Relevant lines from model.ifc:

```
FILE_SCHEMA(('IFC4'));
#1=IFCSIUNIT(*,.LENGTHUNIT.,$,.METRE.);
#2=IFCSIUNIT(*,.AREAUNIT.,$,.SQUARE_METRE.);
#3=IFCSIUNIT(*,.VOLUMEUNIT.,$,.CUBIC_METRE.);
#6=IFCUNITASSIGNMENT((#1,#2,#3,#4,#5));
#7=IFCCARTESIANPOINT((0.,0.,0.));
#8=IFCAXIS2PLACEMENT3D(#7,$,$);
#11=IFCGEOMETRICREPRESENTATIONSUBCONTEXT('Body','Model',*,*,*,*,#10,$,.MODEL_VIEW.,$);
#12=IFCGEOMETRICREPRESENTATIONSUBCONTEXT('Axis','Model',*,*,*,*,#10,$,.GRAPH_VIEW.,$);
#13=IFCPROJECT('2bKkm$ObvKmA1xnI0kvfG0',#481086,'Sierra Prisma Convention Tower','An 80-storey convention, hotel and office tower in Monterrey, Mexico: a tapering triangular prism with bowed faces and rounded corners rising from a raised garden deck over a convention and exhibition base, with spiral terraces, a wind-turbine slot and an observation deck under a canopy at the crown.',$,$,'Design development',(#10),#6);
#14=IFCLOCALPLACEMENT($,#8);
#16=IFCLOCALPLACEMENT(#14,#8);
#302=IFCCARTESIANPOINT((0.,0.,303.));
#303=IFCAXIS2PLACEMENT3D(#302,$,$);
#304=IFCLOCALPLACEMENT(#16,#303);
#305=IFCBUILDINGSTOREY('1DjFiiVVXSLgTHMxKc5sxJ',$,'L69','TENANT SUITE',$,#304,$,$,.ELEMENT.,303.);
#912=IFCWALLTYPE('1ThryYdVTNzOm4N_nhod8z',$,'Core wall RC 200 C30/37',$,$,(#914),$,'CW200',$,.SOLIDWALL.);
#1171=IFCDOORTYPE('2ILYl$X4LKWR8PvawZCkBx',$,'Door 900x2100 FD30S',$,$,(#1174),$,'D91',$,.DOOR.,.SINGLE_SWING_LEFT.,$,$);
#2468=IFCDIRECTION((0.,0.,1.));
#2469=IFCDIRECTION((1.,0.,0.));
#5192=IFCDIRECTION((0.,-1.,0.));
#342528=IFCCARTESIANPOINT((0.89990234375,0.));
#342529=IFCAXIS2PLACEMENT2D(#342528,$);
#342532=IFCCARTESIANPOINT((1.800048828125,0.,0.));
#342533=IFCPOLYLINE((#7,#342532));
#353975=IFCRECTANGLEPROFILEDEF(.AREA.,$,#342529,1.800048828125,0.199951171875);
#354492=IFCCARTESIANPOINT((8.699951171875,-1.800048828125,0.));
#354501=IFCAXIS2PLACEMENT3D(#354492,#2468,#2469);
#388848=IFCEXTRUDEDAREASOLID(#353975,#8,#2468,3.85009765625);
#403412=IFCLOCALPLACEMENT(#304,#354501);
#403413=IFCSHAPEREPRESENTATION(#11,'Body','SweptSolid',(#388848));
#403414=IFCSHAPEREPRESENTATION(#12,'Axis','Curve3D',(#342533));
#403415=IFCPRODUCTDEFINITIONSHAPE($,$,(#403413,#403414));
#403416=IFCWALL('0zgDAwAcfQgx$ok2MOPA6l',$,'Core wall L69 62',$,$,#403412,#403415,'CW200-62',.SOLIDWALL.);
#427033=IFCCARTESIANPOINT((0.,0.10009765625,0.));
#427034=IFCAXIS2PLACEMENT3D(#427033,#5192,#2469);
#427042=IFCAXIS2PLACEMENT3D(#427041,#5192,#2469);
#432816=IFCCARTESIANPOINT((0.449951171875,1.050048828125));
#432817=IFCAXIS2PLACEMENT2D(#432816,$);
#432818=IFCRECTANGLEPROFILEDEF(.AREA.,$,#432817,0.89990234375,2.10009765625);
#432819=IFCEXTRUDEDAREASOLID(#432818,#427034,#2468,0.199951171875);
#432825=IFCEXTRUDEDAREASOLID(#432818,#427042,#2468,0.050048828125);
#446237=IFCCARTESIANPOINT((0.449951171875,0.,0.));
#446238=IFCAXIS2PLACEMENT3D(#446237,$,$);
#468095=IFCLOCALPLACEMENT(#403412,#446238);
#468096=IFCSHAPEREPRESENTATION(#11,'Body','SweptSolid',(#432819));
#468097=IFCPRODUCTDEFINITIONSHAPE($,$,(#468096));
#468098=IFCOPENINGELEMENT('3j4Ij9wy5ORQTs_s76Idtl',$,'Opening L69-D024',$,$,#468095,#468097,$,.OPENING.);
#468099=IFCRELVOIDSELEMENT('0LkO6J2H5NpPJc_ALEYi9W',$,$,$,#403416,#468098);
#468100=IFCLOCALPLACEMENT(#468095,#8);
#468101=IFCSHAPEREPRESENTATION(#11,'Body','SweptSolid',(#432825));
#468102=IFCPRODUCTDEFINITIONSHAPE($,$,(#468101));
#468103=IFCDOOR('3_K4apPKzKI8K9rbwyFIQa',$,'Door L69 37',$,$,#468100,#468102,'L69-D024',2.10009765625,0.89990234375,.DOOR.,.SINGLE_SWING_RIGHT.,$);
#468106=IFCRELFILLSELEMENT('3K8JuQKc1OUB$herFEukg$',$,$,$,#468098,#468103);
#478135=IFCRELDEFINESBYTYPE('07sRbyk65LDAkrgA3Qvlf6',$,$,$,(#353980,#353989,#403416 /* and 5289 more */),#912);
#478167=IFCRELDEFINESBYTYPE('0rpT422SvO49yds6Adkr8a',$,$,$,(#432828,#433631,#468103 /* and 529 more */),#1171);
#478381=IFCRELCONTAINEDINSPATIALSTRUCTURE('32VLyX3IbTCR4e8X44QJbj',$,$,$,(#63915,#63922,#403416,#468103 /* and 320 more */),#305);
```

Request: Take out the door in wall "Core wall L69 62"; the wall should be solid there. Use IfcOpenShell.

```python
import ifcopenshell
import ifcopenshell.api.feature
import ifcopenshell.api.root
import ifcopenshell.geom
import ifcopenshell.util.shape

model = ifcopenshell.open("model.ifc")
settings = ifcopenshell.geom.settings()


def volume(element):
    """Net volume in cubic metres, openings subtracted."""
    shape = ifcopenshell.geom.create_shape(settings, element)
    return ifcopenshell.util.shape.get_volume(shape.geometry)


door = model.by_id(468103)
opening = door.FillsVoids[0].RelatingOpeningElement
wall = opening.VoidsElements[0].RelatingBuildingElement
before = volume(wall)

ifcopenshell.api.root.remove_product(model, product=door)
ifcopenshell.api.feature.remove_feature(model, feature=opening)

after = volume(wall)

print(f"wall volume {before:.3f} -> {after:.3f} m3")

model.write("model_v2.ifc")
```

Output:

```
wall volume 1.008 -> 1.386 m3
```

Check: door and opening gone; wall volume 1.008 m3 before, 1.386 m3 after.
